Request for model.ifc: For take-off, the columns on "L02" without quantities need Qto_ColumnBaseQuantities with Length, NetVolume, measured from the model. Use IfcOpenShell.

First a look at what the model holds.

```python
import ifcopenshell
import ifcopenshell.util.element
import ifcopenshell.util.unit

model = ifcopenshell.open("model.ifc")
print(model.schema)
for unit_type in ("LENGTHUNIT", "AREAUNIT", "VOLUMEUNIT"):
    print(unit_type, ifcopenshell.util.unit.calculate_unit_scale(model, unit_type))
storey = next(s for s in model.by_type("IfcBuildingStorey") if s.Name == "L02")
columns = [e for e in ifcopenshell.util.element.get_decomposition(storey) if e.is_a("IfcColumn")]
for e in sorted(columns, key=lambda e: e.id()):
    print(e.id(), e.is_a(), e.Name, list(ifcopenshell.util.element.get_psets(e, qtos_only=True)), sep=" | ")
```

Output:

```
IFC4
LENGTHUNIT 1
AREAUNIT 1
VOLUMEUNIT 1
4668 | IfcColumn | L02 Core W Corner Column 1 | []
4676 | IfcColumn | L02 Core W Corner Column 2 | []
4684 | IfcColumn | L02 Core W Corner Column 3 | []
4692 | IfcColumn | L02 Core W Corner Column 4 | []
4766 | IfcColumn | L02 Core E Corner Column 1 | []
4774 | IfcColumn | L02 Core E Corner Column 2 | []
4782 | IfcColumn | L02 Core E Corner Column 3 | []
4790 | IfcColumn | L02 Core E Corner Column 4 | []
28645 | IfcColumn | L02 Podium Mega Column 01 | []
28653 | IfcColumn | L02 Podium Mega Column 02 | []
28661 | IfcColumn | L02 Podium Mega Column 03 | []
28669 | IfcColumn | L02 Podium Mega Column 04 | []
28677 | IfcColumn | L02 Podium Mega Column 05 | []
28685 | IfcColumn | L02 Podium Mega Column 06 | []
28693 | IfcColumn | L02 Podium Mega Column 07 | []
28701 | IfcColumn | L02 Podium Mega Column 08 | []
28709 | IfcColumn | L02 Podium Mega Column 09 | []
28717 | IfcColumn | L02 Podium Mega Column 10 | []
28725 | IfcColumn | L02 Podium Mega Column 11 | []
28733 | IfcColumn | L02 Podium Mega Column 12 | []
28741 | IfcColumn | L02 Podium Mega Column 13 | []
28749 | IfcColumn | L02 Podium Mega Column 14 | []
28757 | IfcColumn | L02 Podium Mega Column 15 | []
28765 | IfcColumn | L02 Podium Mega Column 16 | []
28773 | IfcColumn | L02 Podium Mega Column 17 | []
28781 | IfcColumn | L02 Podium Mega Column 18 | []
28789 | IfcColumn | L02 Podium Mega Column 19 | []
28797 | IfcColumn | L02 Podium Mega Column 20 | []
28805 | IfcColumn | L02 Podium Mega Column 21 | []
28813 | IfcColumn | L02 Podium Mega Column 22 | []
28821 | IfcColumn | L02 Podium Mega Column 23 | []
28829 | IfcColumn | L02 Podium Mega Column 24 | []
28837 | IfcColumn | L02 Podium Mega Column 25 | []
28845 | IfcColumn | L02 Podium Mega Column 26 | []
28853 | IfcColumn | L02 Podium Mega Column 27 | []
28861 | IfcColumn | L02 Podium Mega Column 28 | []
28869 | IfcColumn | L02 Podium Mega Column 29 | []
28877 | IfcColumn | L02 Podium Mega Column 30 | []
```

```python
import ifcopenshell
import ifcopenshell.api.pset
import ifcopenshell.geom
import ifcopenshell.util.element
import ifcopenshell.util.shape
import ifcopenshell.util.unit

model = ifcopenshell.open("model.ifc")
unit_scale = ifcopenshell.util.unit.calculate_unit_scale(model)
volume_scale = ifcopenshell.util.unit.calculate_unit_scale(model, "VOLUMEUNIT")
settings = ifcopenshell.geom.settings()

storey = next(s for s in model.by_type("IfcBuildingStorey") if s.Name == "L02")
columns = [e for e in ifcopenshell.util.element.get_decomposition(storey) if e.is_a("IfcColumn")]

for e in sorted(columns, key=lambda e: e.id()):
    if ifcopenshell.util.element.get_psets(e, qtos_only=True, should_inherit=False):
        continue
    # Geometry comes back in metres, in the element's own axes.
    shape = ifcopenshell.geom.create_shape(settings, e)
    values = {
        "Length": ifcopenshell.util.shape.get_z(shape.geometry) / unit_scale,
        "NetVolume": ifcopenshell.util.shape.get_volume(shape.geometry) / volume_scale,
    }
    qto = ifcopenshell.api.pset.add_qto(model, product=e, name="Qto_ColumnBaseQuantities")
    ifcopenshell.api.pset.edit_qto(model, qto=qto, properties=values)
    print(e.id(), {k: round(v, 3) for k, v in values.items()})

model.write("model_v2.ifc")
```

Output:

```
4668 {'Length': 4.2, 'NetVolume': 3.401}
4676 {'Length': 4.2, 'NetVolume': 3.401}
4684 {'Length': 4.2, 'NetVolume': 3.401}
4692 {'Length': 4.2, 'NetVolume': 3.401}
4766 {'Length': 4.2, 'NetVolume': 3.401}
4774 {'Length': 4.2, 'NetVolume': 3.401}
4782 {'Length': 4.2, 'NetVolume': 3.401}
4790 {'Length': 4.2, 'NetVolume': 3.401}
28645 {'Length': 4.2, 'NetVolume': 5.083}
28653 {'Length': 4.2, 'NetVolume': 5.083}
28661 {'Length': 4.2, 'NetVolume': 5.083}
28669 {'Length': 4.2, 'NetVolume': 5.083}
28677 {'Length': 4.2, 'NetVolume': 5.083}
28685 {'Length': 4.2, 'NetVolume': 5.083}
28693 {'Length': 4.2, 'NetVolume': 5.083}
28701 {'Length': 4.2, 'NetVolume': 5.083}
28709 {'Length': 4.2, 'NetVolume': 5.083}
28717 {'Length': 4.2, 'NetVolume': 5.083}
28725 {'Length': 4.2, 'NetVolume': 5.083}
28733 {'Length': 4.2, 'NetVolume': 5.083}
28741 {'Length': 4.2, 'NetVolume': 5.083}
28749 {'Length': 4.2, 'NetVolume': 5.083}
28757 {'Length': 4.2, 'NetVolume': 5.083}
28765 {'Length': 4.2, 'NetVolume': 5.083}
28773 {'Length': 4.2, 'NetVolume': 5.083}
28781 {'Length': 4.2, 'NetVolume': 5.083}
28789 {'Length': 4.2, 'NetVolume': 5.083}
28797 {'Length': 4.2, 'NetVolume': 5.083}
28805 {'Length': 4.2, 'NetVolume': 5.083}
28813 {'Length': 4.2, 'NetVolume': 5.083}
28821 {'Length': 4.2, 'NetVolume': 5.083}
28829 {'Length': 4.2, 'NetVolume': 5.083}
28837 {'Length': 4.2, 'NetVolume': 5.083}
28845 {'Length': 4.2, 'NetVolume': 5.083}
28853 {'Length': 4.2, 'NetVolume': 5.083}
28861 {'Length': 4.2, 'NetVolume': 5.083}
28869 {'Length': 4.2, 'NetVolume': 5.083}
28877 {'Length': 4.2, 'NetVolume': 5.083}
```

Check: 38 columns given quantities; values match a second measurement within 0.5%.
